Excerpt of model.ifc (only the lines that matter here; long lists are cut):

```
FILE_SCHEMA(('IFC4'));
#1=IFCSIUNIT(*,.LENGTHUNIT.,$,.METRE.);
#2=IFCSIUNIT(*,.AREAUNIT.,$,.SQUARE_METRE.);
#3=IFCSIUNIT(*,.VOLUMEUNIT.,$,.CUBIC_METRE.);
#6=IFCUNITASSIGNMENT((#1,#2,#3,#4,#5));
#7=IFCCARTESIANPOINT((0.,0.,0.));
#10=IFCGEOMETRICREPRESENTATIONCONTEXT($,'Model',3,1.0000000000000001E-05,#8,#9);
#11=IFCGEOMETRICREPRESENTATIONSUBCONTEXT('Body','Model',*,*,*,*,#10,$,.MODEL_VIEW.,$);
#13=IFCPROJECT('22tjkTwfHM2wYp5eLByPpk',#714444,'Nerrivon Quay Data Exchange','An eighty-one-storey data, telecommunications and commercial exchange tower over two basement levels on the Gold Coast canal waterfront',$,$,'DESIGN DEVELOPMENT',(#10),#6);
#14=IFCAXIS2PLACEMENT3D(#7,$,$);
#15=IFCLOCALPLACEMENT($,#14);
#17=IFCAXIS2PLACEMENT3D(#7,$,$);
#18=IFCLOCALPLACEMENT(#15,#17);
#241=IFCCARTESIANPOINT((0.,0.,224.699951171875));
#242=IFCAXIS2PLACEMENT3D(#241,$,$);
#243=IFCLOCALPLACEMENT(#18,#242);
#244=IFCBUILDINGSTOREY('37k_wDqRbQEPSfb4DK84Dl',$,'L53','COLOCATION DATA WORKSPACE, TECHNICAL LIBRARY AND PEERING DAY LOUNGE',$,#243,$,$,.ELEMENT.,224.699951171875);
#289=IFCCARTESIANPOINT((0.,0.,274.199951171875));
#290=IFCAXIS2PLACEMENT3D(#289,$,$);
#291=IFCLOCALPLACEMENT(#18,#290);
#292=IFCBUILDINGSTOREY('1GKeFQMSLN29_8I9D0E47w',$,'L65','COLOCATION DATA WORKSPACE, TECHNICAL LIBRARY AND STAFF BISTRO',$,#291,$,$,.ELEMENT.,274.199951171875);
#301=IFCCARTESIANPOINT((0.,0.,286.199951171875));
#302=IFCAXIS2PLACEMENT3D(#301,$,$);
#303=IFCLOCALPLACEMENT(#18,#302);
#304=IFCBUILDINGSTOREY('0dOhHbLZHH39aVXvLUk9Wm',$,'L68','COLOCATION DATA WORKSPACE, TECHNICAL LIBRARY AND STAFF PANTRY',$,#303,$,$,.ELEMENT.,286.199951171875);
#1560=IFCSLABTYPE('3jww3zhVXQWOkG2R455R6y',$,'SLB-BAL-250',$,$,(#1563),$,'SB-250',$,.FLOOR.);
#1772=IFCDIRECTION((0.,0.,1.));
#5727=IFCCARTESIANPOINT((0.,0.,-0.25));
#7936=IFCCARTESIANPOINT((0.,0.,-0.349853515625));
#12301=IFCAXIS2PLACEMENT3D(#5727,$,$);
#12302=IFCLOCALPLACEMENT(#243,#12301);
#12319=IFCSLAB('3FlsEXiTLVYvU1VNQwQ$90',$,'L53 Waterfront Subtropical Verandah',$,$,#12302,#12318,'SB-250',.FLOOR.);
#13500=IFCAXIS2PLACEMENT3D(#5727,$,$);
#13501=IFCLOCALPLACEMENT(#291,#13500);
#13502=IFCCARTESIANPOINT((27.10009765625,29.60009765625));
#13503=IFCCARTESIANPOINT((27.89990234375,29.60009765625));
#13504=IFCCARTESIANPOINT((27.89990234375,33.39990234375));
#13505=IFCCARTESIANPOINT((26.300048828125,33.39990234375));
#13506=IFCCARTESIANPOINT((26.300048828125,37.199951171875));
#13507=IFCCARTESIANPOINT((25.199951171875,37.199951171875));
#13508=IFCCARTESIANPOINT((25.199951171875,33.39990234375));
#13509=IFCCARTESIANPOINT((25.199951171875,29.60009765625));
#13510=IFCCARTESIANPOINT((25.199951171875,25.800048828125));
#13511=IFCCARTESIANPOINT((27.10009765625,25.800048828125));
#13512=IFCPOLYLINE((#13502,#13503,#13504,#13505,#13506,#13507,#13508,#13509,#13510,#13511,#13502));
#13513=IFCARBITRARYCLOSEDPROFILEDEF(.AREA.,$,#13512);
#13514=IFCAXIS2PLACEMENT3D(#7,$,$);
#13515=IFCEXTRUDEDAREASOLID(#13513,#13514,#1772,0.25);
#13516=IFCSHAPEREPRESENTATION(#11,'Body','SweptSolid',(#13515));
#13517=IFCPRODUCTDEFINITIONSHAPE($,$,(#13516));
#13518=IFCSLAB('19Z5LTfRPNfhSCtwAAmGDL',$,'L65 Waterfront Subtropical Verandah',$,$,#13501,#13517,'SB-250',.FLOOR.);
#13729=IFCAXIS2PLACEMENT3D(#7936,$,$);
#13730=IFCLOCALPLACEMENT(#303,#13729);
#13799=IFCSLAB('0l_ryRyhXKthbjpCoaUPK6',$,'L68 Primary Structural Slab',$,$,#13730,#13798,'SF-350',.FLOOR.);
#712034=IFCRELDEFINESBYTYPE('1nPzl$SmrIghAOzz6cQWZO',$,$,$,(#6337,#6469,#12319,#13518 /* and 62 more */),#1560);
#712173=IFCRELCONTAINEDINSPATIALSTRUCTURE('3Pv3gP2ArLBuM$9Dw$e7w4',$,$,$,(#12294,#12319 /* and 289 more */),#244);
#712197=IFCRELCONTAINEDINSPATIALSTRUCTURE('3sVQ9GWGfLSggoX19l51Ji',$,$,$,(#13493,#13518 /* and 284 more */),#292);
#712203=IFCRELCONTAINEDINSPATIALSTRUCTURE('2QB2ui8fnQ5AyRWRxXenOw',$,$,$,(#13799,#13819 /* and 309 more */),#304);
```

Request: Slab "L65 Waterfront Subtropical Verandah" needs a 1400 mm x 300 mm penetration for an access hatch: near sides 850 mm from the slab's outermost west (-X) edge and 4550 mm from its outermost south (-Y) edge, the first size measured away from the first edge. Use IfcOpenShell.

```python
import numpy as np
import ifcopenshell
import ifcopenshell.api.feature
import ifcopenshell.api.geometry
import ifcopenshell.api.root
import ifcopenshell.geom
import ifcopenshell.util.placement
import ifcopenshell.util.representation
import ifcopenshell.util.shape
import ifcopenshell.util.unit

model = ifcopenshell.open("model.ifc")
unit_scale = ifcopenshell.util.unit.calculate_unit_scale(model)
settings = ifcopenshell.geom.settings()


def volume(element):
    """Net volume in cubic metres, openings subtracted."""
    shape = ifcopenshell.geom.create_shape(settings, element)
    return ifcopenshell.util.shape.get_volume(shape.geometry)


slab = model.by_guid("19Z5LTfRPNfhSCtwAAmGDL")
before = volume(slab)

# Extent in the slab's own axes, in metres. The edges named are its -X and -Y sides.
slab_shape = ifcopenshell.geom.create_shape(settings, slab)
vertices = ifcopenshell.util.shape.get_vertices(slab_shape.geometry)
x_min, y_min, bottom = vertices.min(axis=0)
top = vertices[:, 2].max()

opening = ifcopenshell.api.root.create_entity(model, ifc_class="IfcOpeningElement", name="Access hatch opening", predefined_type="OPENING")
context = ifcopenshell.util.representation.get_context(model, "Model", "Body", "MODEL_VIEW")
width, depth = 1.4, 0.3
outline = [(0.0, 0.0), (width, 0.0), (width, depth), (0.0, depth), (0.0, 0.0)]
# Overshoot both faces by 50 mm so the cut is clean.
shape = ifcopenshell.api.geometry.add_slab_representation(
    model, context=context, depth=top - bottom + 0.1, polyline=outline
)
ifcopenshell.api.geometry.assign_representation(model, product=opening, representation=shape)

matrix = ifcopenshell.util.placement.get_local_placement(slab.ObjectPlacement)
matrix[:, 3] = matrix @ np.append(np.array([x_min + 0.85, y_min + 4.55, bottom - 0.05]) / unit_scale, 1.0)
ifcopenshell.api.geometry.edit_object_placement(model, product=opening, matrix=matrix, is_si=False)
ifcopenshell.api.feature.add_feature(model, feature=opening, element=slab)

after = volume(slab)

print(f"slab volume {before:.3f} -> {after:.3f} m3")

model.write("model_updated.ifc")
```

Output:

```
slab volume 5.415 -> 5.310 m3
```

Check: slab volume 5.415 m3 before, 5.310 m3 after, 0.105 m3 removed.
